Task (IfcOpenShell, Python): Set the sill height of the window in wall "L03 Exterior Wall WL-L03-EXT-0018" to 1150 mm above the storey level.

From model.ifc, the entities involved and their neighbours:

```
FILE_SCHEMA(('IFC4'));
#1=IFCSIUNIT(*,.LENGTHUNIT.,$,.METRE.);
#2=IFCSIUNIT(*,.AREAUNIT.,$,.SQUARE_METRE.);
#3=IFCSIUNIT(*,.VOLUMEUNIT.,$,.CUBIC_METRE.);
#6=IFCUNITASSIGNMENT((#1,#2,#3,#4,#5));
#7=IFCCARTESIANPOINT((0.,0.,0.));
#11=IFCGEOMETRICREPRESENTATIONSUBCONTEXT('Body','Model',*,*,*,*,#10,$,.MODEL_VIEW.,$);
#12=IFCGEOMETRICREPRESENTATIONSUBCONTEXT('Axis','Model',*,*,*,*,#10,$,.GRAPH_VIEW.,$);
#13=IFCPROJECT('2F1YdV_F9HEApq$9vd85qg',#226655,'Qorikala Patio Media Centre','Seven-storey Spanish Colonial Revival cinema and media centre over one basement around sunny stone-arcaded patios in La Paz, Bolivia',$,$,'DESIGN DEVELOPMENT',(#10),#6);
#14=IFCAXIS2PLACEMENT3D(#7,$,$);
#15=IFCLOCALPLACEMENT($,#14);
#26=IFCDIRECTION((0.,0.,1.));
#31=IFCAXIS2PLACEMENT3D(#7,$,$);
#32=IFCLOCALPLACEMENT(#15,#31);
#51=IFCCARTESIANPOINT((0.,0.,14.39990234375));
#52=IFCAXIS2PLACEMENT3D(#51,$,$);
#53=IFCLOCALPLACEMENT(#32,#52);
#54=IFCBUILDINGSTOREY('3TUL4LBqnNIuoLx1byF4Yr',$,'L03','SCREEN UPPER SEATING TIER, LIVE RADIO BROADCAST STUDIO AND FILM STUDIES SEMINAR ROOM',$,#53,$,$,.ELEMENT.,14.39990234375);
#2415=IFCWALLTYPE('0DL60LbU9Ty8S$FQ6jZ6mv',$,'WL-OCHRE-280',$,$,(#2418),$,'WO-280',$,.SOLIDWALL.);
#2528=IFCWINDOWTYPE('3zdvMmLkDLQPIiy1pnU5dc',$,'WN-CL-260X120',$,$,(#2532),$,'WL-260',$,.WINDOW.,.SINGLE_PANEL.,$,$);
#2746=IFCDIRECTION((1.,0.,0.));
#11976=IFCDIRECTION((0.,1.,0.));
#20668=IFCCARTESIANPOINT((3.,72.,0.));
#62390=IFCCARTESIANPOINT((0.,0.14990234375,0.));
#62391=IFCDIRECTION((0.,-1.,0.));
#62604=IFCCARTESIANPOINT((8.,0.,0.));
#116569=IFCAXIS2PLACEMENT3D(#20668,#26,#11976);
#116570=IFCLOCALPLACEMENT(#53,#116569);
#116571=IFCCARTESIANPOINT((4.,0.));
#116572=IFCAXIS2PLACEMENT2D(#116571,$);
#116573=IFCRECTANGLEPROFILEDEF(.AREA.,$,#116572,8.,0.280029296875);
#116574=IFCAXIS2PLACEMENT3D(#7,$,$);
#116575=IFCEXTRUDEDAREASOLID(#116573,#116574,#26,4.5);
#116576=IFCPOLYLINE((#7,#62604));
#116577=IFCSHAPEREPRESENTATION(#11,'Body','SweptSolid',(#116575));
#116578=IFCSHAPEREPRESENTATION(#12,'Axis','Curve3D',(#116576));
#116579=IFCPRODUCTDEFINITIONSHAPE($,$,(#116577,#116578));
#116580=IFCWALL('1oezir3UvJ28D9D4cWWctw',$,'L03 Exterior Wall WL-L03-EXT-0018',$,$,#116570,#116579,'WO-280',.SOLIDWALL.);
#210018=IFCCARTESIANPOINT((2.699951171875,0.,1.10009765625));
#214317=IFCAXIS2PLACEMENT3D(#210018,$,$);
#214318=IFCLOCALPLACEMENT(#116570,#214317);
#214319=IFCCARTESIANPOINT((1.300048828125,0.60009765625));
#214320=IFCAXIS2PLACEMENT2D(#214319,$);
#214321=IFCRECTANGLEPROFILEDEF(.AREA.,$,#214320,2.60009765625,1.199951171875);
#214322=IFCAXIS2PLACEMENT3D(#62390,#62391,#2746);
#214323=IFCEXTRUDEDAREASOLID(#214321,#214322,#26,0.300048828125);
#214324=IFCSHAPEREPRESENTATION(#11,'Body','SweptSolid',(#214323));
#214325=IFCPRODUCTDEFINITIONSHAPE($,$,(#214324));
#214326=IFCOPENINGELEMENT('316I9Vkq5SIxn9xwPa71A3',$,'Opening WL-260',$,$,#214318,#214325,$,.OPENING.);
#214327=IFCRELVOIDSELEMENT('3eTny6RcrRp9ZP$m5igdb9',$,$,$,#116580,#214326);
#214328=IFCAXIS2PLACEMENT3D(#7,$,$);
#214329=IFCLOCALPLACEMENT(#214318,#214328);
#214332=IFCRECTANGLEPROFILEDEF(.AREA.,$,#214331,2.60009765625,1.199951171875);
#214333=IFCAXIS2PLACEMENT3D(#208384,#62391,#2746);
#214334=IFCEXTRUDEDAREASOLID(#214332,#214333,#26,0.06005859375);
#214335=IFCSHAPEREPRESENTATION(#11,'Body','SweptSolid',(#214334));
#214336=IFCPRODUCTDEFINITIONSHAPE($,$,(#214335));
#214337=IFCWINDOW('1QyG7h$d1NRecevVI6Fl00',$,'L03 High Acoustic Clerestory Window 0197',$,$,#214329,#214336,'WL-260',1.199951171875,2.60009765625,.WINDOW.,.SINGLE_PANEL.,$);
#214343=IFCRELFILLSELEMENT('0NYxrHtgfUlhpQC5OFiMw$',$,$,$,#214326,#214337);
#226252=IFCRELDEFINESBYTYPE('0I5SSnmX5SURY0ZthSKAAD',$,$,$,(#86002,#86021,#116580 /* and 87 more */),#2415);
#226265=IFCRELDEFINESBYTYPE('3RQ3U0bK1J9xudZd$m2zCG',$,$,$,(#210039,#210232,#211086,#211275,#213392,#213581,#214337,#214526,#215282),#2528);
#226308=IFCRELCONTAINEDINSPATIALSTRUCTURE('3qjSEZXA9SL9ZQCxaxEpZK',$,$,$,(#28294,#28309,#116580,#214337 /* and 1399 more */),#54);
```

```python
import numpy as np
import ifcopenshell
import ifcopenshell.api.geometry
import ifcopenshell.geom
import ifcopenshell.util.element
import ifcopenshell.util.placement
import ifcopenshell.util.shape
import ifcopenshell.util.unit

model = ifcopenshell.open("model.ifc")
unit_scale = ifcopenshell.util.unit.calculate_unit_scale(model)

window = model.by_id(214337)
opening = window.FillsVoids[0].RelatingOpeningElement
storey = ifcopenshell.util.element.get_container(window, ifc_class="IfcBuildingStorey")
level = ifcopenshell.util.placement.get_local_placement(storey.ObjectPlacement)[2, 3]

# The opening's origin need not be at the sill, so measure its lowest point.
shape = ifcopenshell.geom.create_shape(ifcopenshell.geom.settings(), opening)
bottom = ifcopenshell.util.shape.get_shape_bottom_elevation(shape, shape.geometry) / unit_scale
dz = level + 1.15 - bottom

shift = np.array([0.0, 0.0, dz])
# The window is placed relative to its opening, so it follows when the opening moves.
matrix = ifcopenshell.util.placement.get_local_placement(opening.ObjectPlacement)
matrix[:3, 3] += shift
ifcopenshell.api.geometry.edit_object_placement(
    model, product=opening, matrix=matrix, is_si=False, should_transform_children=True
)

print(f"moved by {dz * unit_scale:+.3f} m")

model.write("model_updated.ifc")
```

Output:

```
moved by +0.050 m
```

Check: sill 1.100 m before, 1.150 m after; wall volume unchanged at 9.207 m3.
